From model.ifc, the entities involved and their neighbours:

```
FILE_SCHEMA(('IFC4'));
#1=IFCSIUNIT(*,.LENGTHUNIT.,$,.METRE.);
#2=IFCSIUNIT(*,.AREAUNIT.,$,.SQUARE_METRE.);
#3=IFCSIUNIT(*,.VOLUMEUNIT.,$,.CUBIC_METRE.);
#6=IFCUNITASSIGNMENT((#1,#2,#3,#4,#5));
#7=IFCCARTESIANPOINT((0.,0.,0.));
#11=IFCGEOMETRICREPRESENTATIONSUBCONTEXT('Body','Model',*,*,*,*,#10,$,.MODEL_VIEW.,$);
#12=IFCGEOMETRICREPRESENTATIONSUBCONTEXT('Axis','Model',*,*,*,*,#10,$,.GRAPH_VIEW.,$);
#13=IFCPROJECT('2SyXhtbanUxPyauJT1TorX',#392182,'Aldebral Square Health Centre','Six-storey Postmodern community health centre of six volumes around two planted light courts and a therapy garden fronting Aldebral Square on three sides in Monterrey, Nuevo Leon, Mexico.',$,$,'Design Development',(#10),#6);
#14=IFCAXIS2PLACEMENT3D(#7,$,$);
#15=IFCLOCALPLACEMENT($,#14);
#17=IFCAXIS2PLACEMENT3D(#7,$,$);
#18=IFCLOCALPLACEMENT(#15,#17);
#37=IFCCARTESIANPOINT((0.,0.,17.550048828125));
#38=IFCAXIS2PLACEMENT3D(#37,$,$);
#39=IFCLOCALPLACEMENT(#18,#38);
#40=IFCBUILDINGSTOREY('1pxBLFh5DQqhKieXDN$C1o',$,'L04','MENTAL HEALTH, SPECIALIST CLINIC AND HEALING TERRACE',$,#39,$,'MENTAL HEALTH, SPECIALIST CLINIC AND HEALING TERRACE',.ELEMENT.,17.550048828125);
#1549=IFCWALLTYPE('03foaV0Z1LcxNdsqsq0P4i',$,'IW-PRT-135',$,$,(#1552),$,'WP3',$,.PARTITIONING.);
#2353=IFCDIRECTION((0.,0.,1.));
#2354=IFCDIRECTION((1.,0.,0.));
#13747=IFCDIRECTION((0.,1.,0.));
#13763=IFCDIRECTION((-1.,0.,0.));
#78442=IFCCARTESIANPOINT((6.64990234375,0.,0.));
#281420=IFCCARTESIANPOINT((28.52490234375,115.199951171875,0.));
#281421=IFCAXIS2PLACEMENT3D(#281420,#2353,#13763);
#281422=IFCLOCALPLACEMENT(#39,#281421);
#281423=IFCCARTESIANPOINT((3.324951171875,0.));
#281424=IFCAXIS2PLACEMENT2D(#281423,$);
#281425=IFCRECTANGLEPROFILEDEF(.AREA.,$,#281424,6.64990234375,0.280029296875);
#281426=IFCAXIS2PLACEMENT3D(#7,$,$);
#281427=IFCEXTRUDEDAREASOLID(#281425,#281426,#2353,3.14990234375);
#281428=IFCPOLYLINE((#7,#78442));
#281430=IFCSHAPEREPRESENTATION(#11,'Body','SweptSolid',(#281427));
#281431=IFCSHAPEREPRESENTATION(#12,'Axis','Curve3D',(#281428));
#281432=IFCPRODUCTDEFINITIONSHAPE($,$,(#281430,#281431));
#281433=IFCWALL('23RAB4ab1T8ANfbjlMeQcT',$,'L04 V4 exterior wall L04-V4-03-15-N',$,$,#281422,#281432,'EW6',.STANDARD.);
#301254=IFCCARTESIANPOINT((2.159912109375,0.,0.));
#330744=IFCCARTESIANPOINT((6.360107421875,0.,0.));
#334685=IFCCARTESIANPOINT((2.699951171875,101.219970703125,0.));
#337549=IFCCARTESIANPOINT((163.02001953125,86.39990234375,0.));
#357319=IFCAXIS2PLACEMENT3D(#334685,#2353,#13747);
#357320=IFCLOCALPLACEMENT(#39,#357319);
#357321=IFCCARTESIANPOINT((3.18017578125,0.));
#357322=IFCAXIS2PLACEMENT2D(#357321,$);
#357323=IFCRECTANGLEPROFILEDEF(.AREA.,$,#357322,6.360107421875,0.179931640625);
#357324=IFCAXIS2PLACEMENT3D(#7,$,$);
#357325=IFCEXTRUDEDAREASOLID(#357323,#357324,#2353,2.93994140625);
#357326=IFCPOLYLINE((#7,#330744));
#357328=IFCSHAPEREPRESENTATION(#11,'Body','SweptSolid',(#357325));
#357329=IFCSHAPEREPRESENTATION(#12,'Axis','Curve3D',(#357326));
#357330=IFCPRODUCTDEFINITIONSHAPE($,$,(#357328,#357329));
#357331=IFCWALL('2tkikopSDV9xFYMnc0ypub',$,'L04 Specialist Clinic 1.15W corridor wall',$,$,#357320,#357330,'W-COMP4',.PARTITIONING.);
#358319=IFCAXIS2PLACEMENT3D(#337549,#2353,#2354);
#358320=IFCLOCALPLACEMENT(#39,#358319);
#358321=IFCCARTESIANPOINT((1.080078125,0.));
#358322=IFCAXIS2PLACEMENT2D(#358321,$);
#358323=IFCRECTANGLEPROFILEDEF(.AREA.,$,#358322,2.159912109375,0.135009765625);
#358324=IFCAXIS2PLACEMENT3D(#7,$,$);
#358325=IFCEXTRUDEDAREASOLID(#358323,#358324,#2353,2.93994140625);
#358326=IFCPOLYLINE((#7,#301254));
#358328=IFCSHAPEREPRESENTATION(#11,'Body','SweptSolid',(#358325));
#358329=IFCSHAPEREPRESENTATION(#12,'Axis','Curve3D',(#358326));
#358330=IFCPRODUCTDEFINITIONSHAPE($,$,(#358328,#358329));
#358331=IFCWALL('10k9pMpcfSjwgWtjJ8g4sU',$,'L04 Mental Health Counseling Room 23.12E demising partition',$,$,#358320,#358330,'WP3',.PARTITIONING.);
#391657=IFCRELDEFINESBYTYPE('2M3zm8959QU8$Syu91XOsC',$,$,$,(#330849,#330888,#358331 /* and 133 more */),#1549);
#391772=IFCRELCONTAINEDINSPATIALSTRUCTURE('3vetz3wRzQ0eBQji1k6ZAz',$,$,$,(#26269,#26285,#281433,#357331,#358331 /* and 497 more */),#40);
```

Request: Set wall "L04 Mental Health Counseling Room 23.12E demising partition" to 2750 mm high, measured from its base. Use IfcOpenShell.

```python
import ifcopenshell
import ifcopenshell.geom
import ifcopenshell.util.representation
import ifcopenshell.util.shape
import ifcopenshell.util.unit

model = ifcopenshell.open("model.ifc")
unit_scale = ifcopenshell.util.unit.calculate_unit_scale(model)
settings = ifcopenshell.geom.settings()


def volume(element):
    """Net volume in cubic metres, openings subtracted."""
    shape = ifcopenshell.geom.create_shape(settings, element)
    return ifcopenshell.util.shape.get_volume(shape.geometry)


wall = model.by_guid("10k9pMpcfSjwgWtjJ8g4sU")
before = volume(wall)

body = ifcopenshell.util.representation.get_representation(wall, "Model", "Body")
solid = body.Items[0]
old_height = solid.Depth
solid.Depth = 2.75 / unit_scale
after = volume(wall)

print(f"height {old_height:g} -> {solid.Depth:g}, volume {before:.3f} -> {after:.3f} m3")

model.write("model_updated.ifc")
```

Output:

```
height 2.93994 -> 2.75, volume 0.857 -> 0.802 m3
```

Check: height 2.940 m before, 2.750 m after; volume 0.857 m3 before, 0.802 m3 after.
